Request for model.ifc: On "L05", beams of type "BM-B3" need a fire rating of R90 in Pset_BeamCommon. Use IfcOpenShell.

First a look at what the model holds.

```python
import ifcopenshell
import ifcopenshell.util.element

model = ifcopenshell.open("model.ifc")
print(model.schema)
storey = next(s for s in model.by_type("IfcBuildingStorey") if s.Name == "L05")
beams = [e for e in ifcopenshell.util.element.get_decomposition(storey) if e.is_a("IfcBeam")]
seen = {}
for e in beams:
    element_type = ifcopenshell.util.element.get_type(e)
    key = (element_type.Name if element_type != e and element_type else None, ifcopenshell.util.element.get_pset(e, "Pset_BeamCommon", "FireRating"))
    seen[key] = seen.get(key, 0) + 1
for (name, value), count in sorted(seen.items(), key=str):
    print(count, "x", name, "|", value)
```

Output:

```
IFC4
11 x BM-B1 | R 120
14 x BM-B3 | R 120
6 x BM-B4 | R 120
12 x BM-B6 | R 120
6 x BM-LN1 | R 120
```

```python
import ifcopenshell
import ifcopenshell.api.pset
import ifcopenshell.util.element

model = ifcopenshell.open("model.ifc")

storey = next(s for s in model.by_type("IfcBuildingStorey") if s.Name == "L05")
beams = [e for e in ifcopenshell.util.element.get_decomposition(storey) if e.is_a("IfcBeam")]

count = 0
for e in beams:
    element_type = ifcopenshell.util.element.get_type(e)
    if element_type in (None, e) or element_type.Name != "BM-B3":
        continue
    # add_pset returns the element's existing set when there is one.
    pset = ifcopenshell.api.pset.add_pset(model, product=e, name="Pset_BeamCommon")
    ifcopenshell.api.pset.edit_pset(model, pset=pset, properties={"FireRating": "R90"})
    count += 1

print(count, "beams updated")

model.write("model-out.ifc")
```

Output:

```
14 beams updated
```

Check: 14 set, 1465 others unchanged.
